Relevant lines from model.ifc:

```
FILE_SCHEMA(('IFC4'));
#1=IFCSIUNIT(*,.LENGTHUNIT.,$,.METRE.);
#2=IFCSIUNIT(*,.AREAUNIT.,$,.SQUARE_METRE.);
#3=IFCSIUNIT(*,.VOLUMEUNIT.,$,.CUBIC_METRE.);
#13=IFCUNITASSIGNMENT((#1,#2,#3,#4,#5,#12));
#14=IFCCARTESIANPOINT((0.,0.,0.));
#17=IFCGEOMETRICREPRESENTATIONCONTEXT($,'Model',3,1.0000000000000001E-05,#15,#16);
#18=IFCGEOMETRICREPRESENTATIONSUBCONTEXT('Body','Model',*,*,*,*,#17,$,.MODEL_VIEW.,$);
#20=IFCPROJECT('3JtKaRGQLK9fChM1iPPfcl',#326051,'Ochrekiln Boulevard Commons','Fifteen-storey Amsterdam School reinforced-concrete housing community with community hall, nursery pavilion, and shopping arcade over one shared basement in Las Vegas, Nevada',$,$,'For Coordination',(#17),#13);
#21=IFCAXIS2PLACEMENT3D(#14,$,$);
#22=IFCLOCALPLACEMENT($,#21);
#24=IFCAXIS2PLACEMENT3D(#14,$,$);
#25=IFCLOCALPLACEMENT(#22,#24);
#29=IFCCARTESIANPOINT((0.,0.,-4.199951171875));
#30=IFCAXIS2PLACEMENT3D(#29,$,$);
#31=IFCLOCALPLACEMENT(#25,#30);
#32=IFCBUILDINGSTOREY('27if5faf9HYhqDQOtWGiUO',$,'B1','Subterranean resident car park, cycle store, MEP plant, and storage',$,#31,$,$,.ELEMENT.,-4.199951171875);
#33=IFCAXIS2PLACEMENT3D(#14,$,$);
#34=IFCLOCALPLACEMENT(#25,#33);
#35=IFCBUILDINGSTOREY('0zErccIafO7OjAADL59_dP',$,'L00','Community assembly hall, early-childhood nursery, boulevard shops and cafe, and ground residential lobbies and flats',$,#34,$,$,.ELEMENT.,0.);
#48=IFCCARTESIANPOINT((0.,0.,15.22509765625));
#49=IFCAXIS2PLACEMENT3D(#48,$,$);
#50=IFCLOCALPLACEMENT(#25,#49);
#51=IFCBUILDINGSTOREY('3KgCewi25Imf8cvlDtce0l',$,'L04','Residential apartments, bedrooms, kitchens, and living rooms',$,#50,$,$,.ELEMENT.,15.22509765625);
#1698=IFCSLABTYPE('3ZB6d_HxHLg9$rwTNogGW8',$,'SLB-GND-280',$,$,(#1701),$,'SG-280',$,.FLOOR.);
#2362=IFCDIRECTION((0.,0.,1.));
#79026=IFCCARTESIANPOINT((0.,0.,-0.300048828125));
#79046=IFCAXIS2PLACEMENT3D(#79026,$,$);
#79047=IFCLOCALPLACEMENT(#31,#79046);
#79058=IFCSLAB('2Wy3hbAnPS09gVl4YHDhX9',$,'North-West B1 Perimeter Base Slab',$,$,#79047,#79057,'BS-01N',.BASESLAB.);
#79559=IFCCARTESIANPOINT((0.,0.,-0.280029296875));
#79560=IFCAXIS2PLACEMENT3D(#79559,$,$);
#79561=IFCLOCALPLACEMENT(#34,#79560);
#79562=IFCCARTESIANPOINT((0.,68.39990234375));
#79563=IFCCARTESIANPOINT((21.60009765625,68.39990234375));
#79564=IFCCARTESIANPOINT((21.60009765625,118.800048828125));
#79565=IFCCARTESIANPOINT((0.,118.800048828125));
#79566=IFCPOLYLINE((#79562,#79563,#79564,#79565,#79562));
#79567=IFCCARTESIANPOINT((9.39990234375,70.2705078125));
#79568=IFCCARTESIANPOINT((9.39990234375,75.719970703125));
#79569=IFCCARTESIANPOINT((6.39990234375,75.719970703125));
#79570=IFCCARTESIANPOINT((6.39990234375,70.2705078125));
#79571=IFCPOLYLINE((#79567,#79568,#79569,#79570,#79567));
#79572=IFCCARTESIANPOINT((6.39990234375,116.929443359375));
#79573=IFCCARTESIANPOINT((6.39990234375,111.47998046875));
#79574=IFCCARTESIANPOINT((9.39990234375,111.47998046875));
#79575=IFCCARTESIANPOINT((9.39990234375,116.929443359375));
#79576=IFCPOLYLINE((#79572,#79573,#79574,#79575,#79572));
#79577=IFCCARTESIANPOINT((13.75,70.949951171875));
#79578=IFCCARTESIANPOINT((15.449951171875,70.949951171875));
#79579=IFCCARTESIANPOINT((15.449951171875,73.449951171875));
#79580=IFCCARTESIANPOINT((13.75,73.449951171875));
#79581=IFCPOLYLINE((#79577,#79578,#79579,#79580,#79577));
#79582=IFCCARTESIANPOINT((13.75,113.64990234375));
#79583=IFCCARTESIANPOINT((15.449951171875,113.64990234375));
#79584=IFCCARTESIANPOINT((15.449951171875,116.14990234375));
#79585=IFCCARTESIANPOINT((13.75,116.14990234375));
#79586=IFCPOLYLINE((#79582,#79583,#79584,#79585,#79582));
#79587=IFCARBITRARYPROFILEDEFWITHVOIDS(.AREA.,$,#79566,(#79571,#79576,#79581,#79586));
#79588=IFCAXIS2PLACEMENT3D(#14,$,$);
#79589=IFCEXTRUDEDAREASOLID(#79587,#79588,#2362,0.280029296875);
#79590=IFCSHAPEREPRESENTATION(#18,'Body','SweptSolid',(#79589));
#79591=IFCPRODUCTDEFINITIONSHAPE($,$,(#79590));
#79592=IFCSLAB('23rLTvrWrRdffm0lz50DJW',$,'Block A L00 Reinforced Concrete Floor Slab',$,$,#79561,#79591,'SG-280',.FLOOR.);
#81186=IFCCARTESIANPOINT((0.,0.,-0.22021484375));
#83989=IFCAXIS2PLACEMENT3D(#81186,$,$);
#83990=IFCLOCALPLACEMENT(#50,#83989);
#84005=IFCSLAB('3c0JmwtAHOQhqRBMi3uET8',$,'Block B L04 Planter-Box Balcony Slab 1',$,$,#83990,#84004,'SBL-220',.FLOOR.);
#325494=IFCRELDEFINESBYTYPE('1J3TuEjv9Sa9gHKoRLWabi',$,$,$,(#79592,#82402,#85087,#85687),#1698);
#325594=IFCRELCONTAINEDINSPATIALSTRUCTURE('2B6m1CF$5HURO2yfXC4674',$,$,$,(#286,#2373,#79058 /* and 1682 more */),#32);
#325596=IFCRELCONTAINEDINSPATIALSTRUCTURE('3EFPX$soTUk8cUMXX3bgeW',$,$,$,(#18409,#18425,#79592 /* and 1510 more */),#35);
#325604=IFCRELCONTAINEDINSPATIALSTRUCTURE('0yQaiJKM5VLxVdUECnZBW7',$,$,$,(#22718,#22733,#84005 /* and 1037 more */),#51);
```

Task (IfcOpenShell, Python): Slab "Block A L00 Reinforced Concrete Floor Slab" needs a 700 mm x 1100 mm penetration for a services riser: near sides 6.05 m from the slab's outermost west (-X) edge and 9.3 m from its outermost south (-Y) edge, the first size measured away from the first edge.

```python
import numpy as np
import ifcopenshell
import ifcopenshell.api.feature
import ifcopenshell.api.geometry
import ifcopenshell.api.root
import ifcopenshell.geom
import ifcopenshell.util.placement
import ifcopenshell.util.representation
import ifcopenshell.util.shape
import ifcopenshell.util.unit

model = ifcopenshell.open("model.ifc")
unit_scale = ifcopenshell.util.unit.calculate_unit_scale(model)
settings = ifcopenshell.geom.settings()


def volume(element):
    """Net volume in cubic metres, openings subtracted."""
    shape = ifcopenshell.geom.create_shape(settings, element)
    return ifcopenshell.util.shape.get_volume(shape.geometry)


slab = model.by_id(79592)
before = volume(slab)

# Extent in the slab's own axes, in metres. The edges named are its -X and -Y sides.
slab_shape = ifcopenshell.geom.create_shape(settings, slab)
vertices = ifcopenshell.util.shape.get_vertices(slab_shape.geometry)
x_min, y_min, bottom = vertices.min(axis=0)
top = vertices[:, 2].max()

opening = ifcopenshell.api.root.create_entity(model, ifc_class="IfcOpeningElement", name="Services riser opening", predefined_type="OPENING")
context = ifcopenshell.util.representation.get_context(model, "Model", "Body", "MODEL_VIEW")
width, depth = 0.7, 1.1
outline = [(0.0, 0.0), (width, 0.0), (width, depth), (0.0, depth), (0.0, 0.0)]
# Overshoot both faces by 50 mm so the cut is clean.
shape = ifcopenshell.api.geometry.add_slab_representation(
    model, context=context, depth=top - bottom + 0.1, polyline=outline
)
ifcopenshell.api.geometry.assign_representation(model, product=opening, representation=shape)

matrix = ifcopenshell.util.placement.get_local_placement(slab.ObjectPlacement)
matrix[:, 3] = matrix @ np.append(np.array([x_min + 6.05, y_min + 9.3, bottom - 0.05]) / unit_scale, 1.0)
ifcopenshell.api.geometry.edit_object_placement(model, product=opening, matrix=matrix, is_si=False)
ifcopenshell.api.feature.add_feature(model, feature=opening, element=slab)

after = volume(slab)

print(f"slab volume {before:.3f} -> {after:.3f} m3")

model.write("model_rev.ifc")
```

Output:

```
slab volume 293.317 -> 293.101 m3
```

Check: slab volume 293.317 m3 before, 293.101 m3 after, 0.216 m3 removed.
